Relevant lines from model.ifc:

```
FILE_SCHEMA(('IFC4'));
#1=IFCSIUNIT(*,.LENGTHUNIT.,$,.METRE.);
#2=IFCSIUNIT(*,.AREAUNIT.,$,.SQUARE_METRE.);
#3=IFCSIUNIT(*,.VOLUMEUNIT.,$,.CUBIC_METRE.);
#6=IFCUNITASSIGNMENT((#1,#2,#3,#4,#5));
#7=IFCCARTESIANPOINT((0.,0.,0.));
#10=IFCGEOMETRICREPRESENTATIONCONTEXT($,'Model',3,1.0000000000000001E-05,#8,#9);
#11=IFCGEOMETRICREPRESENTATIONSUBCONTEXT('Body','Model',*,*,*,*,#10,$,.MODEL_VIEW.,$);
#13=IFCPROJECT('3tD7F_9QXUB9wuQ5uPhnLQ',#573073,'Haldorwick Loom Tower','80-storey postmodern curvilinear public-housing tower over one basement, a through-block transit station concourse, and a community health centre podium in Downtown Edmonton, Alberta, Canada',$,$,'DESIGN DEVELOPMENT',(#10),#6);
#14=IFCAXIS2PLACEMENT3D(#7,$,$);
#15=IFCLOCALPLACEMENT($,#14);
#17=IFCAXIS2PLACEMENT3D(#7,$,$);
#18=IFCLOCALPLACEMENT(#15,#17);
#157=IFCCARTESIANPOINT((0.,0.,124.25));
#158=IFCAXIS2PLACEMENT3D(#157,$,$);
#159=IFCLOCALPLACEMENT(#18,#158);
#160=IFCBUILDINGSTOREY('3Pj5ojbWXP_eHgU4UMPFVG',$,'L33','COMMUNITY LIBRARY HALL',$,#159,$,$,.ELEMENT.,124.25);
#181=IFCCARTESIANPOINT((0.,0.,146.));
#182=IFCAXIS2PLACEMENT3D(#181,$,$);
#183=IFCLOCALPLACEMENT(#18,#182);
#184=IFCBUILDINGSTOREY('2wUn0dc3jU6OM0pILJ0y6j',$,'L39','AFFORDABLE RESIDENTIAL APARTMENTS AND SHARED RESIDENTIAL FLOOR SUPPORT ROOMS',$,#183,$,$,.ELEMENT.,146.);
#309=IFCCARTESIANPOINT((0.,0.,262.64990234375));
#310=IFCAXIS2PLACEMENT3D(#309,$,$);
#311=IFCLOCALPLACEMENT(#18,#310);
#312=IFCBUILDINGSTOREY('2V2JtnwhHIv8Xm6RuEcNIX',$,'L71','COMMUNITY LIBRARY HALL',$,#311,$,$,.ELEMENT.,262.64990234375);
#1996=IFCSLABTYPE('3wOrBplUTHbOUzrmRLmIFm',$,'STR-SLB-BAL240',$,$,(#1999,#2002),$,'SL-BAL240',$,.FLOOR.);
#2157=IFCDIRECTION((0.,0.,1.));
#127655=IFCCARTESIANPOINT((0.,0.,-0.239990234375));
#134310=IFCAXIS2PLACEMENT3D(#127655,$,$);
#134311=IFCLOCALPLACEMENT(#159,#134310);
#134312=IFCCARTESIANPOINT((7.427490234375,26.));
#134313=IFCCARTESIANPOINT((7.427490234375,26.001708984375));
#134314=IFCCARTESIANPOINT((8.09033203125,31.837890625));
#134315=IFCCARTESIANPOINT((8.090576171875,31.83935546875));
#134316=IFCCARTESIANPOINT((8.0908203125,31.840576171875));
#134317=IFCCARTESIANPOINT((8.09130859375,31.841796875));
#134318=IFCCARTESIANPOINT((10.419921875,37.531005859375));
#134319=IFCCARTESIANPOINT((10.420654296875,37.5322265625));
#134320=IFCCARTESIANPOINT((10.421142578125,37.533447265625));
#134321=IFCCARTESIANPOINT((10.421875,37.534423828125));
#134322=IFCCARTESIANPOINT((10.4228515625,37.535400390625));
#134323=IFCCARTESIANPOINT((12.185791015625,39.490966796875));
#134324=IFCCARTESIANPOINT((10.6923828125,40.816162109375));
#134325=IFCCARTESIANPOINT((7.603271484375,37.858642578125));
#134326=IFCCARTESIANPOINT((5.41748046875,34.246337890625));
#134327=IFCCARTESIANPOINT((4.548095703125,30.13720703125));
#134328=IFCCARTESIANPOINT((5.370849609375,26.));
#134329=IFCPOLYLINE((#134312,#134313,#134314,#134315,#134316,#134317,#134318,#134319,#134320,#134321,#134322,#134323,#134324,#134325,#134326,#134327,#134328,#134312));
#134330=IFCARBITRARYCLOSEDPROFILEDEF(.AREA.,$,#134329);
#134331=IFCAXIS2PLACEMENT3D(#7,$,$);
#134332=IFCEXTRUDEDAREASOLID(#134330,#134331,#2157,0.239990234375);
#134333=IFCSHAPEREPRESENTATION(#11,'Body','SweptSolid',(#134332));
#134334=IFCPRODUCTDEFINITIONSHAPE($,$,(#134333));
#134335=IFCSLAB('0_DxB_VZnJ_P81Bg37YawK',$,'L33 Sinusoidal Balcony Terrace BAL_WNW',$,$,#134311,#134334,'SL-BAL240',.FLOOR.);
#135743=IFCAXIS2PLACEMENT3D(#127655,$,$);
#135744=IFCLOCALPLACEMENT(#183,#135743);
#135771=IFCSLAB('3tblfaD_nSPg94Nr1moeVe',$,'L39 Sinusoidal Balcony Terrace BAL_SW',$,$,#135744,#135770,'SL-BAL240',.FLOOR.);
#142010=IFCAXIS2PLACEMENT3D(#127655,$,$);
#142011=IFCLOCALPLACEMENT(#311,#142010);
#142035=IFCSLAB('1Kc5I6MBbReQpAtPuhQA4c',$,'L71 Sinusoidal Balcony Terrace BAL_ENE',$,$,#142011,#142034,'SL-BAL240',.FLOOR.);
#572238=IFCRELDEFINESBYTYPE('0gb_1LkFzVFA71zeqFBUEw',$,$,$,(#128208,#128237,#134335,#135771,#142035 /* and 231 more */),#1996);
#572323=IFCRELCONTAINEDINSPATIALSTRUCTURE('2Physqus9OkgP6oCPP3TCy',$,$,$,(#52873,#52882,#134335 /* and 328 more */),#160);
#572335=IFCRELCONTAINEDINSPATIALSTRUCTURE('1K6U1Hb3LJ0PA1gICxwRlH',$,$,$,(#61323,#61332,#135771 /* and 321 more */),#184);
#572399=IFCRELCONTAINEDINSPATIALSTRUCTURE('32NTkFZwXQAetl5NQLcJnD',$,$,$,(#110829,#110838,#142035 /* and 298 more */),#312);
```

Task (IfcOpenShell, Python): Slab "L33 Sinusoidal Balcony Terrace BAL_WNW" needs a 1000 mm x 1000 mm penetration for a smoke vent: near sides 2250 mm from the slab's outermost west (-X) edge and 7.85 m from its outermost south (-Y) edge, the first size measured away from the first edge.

```python
import numpy as np
import ifcopenshell
import ifcopenshell.api.feature
import ifcopenshell.api.geometry
import ifcopenshell.api.root
import ifcopenshell.geom
import ifcopenshell.util.placement
import ifcopenshell.util.representation
import ifcopenshell.util.shape
import ifcopenshell.util.unit

model = ifcopenshell.open("model.ifc")
unit_scale = ifcopenshell.util.unit.calculate_unit_scale(model)
settings = ifcopenshell.geom.settings()


def volume(element):
    """Net volume in cubic metres, openings subtracted."""
    shape = ifcopenshell.geom.create_shape(settings, element)
    return ifcopenshell.util.shape.get_volume(shape.geometry)


slab = model.by_guid("0_DxB_VZnJ_P81Bg37YawK")
before = volume(slab)

# Extent in the slab's own axes, in metres. The edges named are its -X and -Y sides.
slab_shape = ifcopenshell.geom.create_shape(settings, slab)
vertices = ifcopenshell.util.shape.get_vertices(slab_shape.geometry)
x_min, y_min, bottom = vertices.min(axis=0)
top = vertices[:, 2].max()

opening = ifcopenshell.api.root.create_entity(model, ifc_class="IfcOpeningElement", name="Smoke vent opening", predefined_type="OPENING")
context = ifcopenshell.util.representation.get_context(model, "Model", "Body", "MODEL_VIEW")
width, depth = 1, 1
outline = [(0.0, 0.0), (width, 0.0), (width, depth), (0.0, depth), (0.0, 0.0)]
# Overshoot both faces by 50 mm so the cut is clean.
shape = ifcopenshell.api.geometry.add_slab_representation(
    model, context=context, depth=top - bottom + 0.1, polyline=outline
)
ifcopenshell.api.geometry.assign_representation(model, product=opening, representation=shape)

matrix = ifcopenshell.util.placement.get_local_placement(slab.ObjectPlacement)
matrix[:, 3] = matrix @ np.append(np.array([x_min + 2.25, y_min + 7.85, bottom - 0.05]) / unit_scale, 1.0)
ifcopenshell.api.geometry.edit_object_placement(model, product=opening, matrix=matrix, is_si=False)
ifcopenshell.api.feature.add_feature(model, feature=opening, element=slab)

after = volume(slab)

print(f"slab volume {before:.3f} -> {after:.3f} m3")

model.write("model_v2.ifc")
```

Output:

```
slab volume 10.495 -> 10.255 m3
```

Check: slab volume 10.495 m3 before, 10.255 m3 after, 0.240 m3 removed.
